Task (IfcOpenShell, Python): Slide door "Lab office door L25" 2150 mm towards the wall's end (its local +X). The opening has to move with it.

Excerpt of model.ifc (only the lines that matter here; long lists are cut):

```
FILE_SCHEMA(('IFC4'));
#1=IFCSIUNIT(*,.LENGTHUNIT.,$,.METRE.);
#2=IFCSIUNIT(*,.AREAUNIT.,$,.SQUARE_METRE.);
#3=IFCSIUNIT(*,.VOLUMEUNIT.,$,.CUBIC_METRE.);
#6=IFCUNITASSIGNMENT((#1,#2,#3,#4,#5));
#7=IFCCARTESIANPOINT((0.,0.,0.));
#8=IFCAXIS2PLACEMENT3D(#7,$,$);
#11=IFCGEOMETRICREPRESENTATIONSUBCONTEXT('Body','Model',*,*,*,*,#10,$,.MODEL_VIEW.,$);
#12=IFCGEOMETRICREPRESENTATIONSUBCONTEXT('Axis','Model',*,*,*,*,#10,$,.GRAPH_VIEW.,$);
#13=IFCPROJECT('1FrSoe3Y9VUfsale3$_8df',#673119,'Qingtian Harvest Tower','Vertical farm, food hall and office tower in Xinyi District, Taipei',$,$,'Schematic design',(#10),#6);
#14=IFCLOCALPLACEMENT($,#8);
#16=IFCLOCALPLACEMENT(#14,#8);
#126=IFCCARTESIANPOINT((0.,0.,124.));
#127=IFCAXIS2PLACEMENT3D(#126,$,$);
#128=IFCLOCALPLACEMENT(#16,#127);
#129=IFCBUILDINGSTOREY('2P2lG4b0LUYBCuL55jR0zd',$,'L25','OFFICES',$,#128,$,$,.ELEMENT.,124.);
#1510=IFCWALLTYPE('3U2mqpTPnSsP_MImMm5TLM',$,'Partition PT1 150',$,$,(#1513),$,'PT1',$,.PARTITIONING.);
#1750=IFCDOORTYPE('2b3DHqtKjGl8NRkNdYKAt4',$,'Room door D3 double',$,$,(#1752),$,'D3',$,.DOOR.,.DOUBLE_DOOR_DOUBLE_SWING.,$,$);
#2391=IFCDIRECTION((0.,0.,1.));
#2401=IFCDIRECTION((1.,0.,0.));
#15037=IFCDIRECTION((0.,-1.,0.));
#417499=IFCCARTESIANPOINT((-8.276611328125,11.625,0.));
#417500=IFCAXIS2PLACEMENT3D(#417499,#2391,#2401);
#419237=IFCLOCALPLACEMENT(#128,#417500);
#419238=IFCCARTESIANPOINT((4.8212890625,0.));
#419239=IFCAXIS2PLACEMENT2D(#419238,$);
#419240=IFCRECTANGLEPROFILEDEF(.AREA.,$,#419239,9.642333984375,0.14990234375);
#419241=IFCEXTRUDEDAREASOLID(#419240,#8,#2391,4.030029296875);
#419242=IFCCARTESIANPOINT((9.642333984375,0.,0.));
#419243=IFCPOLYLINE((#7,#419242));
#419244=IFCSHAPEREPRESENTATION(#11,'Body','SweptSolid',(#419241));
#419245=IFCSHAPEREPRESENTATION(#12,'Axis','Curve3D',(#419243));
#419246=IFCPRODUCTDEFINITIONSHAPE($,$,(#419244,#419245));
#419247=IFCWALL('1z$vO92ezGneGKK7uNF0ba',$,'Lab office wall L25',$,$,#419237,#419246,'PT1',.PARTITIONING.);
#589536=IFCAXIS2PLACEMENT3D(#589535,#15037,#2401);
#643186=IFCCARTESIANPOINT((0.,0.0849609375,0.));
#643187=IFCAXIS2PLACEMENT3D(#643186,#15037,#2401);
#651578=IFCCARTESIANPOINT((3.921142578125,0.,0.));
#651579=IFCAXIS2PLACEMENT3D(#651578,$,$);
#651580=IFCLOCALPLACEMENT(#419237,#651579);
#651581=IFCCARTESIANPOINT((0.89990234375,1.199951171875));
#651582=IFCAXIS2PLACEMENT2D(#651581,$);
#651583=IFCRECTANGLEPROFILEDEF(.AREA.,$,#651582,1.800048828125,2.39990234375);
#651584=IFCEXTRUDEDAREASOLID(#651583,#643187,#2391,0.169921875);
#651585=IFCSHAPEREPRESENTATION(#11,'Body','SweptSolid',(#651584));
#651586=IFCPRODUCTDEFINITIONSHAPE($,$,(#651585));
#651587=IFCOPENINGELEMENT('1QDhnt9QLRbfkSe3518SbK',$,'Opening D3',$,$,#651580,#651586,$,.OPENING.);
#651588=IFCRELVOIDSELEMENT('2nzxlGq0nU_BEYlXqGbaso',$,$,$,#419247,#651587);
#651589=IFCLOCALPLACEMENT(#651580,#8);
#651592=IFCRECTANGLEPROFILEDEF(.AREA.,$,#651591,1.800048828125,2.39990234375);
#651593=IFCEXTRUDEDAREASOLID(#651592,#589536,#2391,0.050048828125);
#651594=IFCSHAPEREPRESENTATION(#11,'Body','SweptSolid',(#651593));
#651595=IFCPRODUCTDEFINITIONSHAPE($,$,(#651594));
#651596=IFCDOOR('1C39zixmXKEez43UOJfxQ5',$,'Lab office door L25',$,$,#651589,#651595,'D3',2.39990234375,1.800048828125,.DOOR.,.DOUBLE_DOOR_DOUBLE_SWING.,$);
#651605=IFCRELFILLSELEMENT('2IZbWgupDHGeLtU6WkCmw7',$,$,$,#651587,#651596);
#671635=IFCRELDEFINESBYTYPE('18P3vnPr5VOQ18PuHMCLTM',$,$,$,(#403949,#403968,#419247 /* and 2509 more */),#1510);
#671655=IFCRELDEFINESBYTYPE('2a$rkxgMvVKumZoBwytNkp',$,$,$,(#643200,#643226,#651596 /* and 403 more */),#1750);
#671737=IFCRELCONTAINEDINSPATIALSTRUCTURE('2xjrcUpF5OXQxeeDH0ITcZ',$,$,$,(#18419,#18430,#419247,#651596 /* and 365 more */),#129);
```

```python
import ifcopenshell
import ifcopenshell.api.geometry
import ifcopenshell.util.placement
import ifcopenshell.util.unit

model = ifcopenshell.open("model.ifc")
unit_scale = ifcopenshell.util.unit.calculate_unit_scale(model)

door = model.by_guid("1C39zixmXKEez43UOJfxQ5")
opening = door.FillsVoids[0].RelatingOpeningElement
wall = opening.VoidsElements[0].RelatingBuildingElement

wall_matrix = ifcopenshell.util.placement.get_local_placement(wall.ObjectPlacement)
shift = wall_matrix[:3, 0] * 2.15 / unit_scale
before = ifcopenshell.util.placement.get_local_placement(door.ObjectPlacement)[:3, 3].copy()

# The door is placed relative to its opening, so it follows when the opening moves.
matrix = ifcopenshell.util.placement.get_local_placement(opening.ObjectPlacement)
matrix[:3, 3] += shift
ifcopenshell.api.geometry.edit_object_placement(
    model, product=opening, matrix=matrix, is_si=False, should_transform_children=True
)

after = ifcopenshell.util.placement.get_local_placement(door.ObjectPlacement)[:3, 3]
print("door moved by", (after - before).round(3) + 0.0)

model.write("model_v2.ifc")
```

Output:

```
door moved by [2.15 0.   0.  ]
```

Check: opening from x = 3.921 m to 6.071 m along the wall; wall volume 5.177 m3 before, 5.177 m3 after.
